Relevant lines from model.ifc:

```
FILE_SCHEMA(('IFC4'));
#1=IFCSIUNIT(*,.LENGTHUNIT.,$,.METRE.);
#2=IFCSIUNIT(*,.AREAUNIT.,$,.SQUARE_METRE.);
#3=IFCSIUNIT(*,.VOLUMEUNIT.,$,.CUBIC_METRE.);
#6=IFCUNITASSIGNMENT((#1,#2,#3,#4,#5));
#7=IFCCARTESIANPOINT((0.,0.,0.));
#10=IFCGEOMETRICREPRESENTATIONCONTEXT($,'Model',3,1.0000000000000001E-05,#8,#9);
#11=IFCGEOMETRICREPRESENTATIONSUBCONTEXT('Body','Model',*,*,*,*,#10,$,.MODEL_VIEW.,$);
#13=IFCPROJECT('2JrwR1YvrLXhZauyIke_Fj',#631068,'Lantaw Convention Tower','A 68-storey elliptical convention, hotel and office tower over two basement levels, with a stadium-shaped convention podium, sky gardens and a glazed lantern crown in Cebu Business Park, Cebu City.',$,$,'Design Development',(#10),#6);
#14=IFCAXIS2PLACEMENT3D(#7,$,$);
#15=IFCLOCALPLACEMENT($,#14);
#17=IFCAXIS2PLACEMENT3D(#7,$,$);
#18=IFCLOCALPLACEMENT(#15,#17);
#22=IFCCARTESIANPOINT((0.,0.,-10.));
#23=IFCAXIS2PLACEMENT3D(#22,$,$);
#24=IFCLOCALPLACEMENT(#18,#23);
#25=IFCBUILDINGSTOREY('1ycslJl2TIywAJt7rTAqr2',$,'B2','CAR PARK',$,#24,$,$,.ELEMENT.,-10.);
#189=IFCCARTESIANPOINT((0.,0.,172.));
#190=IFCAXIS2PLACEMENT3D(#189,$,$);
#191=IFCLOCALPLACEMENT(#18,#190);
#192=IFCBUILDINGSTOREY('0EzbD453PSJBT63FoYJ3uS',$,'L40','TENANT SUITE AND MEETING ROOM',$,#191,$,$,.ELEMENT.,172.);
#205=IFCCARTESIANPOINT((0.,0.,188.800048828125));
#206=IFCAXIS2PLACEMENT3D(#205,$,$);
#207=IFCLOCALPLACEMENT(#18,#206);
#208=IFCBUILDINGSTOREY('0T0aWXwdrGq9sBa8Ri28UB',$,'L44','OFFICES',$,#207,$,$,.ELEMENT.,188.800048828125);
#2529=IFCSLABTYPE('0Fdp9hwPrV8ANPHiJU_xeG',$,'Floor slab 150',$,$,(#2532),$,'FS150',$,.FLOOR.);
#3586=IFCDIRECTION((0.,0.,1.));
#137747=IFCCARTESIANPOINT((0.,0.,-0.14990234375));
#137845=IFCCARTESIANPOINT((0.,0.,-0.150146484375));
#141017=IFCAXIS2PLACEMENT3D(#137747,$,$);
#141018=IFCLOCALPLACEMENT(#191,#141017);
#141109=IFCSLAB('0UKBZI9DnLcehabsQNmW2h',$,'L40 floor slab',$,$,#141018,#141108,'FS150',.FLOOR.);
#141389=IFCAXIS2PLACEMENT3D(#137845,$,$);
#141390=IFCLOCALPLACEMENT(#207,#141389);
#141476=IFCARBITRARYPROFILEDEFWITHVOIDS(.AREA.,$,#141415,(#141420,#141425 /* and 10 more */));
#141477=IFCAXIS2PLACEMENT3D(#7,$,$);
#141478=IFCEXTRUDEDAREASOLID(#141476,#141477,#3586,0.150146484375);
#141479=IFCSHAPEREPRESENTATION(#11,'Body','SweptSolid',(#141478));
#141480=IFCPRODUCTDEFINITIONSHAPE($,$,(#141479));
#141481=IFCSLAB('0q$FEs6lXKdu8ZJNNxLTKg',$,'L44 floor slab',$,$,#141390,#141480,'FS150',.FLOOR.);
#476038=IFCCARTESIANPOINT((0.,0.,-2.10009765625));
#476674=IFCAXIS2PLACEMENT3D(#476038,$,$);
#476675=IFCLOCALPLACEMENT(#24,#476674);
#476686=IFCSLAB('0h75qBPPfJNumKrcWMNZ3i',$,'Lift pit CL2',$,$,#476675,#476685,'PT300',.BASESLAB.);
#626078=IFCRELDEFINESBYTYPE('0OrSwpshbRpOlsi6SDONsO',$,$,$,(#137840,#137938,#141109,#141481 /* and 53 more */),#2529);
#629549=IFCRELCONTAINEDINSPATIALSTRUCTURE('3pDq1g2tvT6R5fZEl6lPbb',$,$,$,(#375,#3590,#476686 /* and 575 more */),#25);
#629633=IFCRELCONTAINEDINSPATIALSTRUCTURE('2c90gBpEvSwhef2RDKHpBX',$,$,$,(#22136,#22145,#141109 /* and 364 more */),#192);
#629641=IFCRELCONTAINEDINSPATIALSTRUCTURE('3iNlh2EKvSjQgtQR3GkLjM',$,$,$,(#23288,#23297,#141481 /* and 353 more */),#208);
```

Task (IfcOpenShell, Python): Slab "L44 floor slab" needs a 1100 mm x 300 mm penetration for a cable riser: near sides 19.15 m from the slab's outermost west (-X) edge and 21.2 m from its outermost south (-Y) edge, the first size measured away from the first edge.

```python
import numpy as np
import ifcopenshell
import ifcopenshell.api.feature
import ifcopenshell.api.geometry
import ifcopenshell.api.root
import ifcopenshell.geom
import ifcopenshell.util.placement
import ifcopenshell.util.representation
import ifcopenshell.util.shape
import ifcopenshell.util.unit

model = ifcopenshell.open("model.ifc")
unit_scale = ifcopenshell.util.unit.calculate_unit_scale(model)
settings = ifcopenshell.geom.settings()


def volume(element):
    """Net volume in cubic metres, openings subtracted."""
    shape = ifcopenshell.geom.create_shape(settings, element)
    return ifcopenshell.util.shape.get_volume(shape.geometry)


slab = model.by_guid("0q$FEs6lXKdu8ZJNNxLTKg")
before = volume(slab)

# Extent in the slab's own axes, in metres. The edges named are its -X and -Y sides.
slab_shape = ifcopenshell.geom.create_shape(settings, slab)
vertices = ifcopenshell.util.shape.get_vertices(slab_shape.geometry)
x_min, y_min, bottom = vertices.min(axis=0)
top = vertices[:, 2].max()

opening = ifcopenshell.api.root.create_entity(model, ifc_class="IfcOpeningElement", name="Cable riser opening", predefined_type="OPENING")
context = ifcopenshell.util.representation.get_context(model, "Model", "Body", "MODEL_VIEW")
width, depth = 1.1, 0.3
outline = [(0.0, 0.0), (width, 0.0), (width, depth), (0.0, depth), (0.0, 0.0)]
# Overshoot both faces by 50 mm so the cut is clean.
shape = ifcopenshell.api.geometry.add_slab_representation(
    model, context=context, depth=top - bottom + 0.1, polyline=outline
)
ifcopenshell.api.geometry.assign_representation(model, product=opening, representation=shape)

matrix = ifcopenshell.util.placement.get_local_placement(slab.ObjectPlacement)
matrix[:, 3] = matrix @ np.append(np.array([x_min + 19.15, y_min + 21.2, bottom - 0.05]) / unit_scale, 1.0)
ifcopenshell.api.geometry.edit_object_placement(model, product=opening, matrix=matrix, is_si=False)
ifcopenshell.api.feature.add_feature(model, feature=opening, element=slab)

after = volume(slab)

print(f"slab volume {before:.3f} -> {after:.3f} m3")

model.write("model-out.ifc")
```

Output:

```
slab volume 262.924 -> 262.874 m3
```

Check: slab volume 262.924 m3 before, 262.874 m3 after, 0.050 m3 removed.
